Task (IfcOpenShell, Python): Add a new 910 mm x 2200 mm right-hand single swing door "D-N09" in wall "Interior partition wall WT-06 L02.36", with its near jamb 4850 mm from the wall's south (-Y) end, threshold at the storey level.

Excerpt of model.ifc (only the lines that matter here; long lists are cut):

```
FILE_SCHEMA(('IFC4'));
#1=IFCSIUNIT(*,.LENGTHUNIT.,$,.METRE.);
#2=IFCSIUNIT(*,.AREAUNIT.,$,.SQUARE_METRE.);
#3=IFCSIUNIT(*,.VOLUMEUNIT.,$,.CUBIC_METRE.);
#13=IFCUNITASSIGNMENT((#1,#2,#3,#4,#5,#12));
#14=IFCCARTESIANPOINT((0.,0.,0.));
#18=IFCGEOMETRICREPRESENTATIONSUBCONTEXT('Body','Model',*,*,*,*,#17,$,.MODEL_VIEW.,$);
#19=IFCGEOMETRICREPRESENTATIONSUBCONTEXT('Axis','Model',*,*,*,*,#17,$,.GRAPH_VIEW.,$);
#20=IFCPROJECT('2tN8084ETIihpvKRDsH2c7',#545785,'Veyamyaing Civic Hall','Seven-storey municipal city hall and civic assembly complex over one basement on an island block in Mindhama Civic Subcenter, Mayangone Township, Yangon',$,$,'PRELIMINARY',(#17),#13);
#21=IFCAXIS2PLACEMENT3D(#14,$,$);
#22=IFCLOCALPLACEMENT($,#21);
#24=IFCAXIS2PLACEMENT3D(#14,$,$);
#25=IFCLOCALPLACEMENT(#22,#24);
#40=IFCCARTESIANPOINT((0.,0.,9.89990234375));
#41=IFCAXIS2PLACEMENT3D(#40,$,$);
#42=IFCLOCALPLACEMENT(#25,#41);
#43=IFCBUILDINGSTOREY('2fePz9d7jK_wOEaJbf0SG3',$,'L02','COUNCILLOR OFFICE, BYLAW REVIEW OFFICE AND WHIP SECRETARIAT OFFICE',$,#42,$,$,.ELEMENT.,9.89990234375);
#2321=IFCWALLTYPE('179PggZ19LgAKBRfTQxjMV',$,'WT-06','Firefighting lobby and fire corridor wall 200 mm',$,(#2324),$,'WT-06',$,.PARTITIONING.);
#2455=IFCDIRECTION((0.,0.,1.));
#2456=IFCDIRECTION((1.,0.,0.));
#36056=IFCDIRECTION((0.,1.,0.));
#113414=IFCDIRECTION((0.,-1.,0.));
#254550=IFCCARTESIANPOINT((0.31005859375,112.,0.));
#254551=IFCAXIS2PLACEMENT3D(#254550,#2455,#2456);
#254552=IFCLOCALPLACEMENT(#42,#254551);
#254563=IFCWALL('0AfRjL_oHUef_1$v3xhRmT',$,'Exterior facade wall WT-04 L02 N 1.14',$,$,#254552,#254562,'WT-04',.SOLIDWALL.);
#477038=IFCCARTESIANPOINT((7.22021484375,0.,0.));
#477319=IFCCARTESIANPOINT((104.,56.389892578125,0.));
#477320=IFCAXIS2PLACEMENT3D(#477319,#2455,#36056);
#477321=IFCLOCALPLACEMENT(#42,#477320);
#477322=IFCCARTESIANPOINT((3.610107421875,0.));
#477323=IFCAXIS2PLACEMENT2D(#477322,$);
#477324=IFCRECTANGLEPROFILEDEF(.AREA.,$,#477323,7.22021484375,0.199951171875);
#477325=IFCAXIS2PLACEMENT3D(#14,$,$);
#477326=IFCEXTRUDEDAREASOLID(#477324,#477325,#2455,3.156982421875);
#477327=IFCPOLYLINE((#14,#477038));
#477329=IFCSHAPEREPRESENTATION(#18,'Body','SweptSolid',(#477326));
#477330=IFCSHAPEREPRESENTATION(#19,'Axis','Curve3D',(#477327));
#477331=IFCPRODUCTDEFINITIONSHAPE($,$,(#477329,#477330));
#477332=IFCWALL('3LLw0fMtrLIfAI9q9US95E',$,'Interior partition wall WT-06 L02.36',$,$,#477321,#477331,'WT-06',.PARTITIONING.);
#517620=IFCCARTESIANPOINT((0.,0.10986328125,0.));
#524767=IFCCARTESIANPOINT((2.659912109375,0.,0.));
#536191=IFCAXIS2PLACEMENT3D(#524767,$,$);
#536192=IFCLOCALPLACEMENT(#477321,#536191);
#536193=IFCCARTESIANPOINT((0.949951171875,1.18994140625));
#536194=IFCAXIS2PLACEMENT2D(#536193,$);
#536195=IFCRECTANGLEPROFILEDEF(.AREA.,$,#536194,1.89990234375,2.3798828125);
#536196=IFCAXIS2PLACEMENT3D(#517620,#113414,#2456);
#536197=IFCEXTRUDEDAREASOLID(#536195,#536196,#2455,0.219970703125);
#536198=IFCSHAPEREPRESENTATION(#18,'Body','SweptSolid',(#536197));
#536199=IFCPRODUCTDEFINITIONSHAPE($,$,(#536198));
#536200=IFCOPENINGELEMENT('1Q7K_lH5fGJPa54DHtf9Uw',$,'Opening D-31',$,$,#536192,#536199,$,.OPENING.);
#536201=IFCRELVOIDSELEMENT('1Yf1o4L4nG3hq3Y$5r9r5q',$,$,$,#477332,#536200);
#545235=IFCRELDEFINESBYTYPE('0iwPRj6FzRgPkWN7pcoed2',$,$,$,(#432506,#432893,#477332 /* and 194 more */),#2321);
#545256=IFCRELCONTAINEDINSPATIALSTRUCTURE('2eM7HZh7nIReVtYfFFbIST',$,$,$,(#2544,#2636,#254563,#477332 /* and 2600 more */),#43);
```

```python
import numpy as np
import ifcopenshell
import ifcopenshell.api.feature
import ifcopenshell.api.geometry
import ifcopenshell.api.root
import ifcopenshell.api.spatial
import ifcopenshell.geom
import ifcopenshell.util.element
import ifcopenshell.util.placement
import ifcopenshell.util.representation
import ifcopenshell.util.shape
import ifcopenshell.util.unit

model = ifcopenshell.open("model.ifc")
unit_scale = ifcopenshell.util.unit.calculate_unit_scale(model)
settings = ifcopenshell.geom.settings()


def volume(element):
    """Net volume in cubic metres, openings subtracted."""
    shape = ifcopenshell.geom.create_shape(settings, element)
    return ifcopenshell.util.shape.get_volume(shape.geometry)


wall = model.by_id(477332)
storey = ifcopenshell.util.element.get_container(wall, ifc_class="IfcBuildingStorey")
context = ifcopenshell.util.representation.get_context(model, "Model", "Body", "MODEL_VIEW")
before = volume(wall)

width, height, from_end, sill = 0.91, 2.2, 4.85, 0.0  # metres

# The wall runs along its own X axis, and the end named is its -X end.
wall_shape = ifcopenshell.geom.create_shape(settings, wall)
x, y, z = ifcopenshell.util.shape.get_vertices(wall_shape.geometry).T
start = x.min() + from_end
face, thickness = float(y.min()), float(y.max() - y.min())
wall_matrix = ifcopenshell.util.placement.get_local_placement(wall.ObjectPlacement)
level = ifcopenshell.util.placement.get_local_placement(storey.ObjectPlacement)[2, 3]


def in_wall(x, y):
    """Placement at x, y metres in the wall's axes, at sill height."""
    matrix = wall_matrix.copy()
    matrix[:, 3] = wall_matrix @ np.array([x / unit_scale, y / unit_scale, 0.0, 1.0])
    matrix[2, 3] = level + sill / unit_scale
    return matrix


# Opening: a box that overshoots both wall faces by 50 mm.
opening = ifcopenshell.api.root.create_entity(model, ifc_class="IfcOpeningElement", predefined_type="OPENING")
box = ifcopenshell.api.geometry.add_wall_representation(
    model, context=context, length=width, height=height, thickness=thickness + 0.1
)
ifcopenshell.api.geometry.assign_representation(model, product=opening, representation=box)
ifcopenshell.api.geometry.edit_object_placement(model, product=opening, matrix=in_wall(start, face - 0.05), is_si=False)
ifcopenshell.api.feature.add_feature(model, feature=opening, element=wall)

door = ifcopenshell.api.root.create_entity(model, ifc_class="IfcDoor", name="D-N09", predefined_type="DOOR")
door.OverallWidth, door.OverallHeight = width / unit_scale, height / unit_scale
door.OperationType = "SINGLE_SWING_RIGHT"
body = ifcopenshell.api.geometry.add_door_representation(
    model,
    context=context,
    overall_width=door.OverallWidth,
    overall_height=door.OverallHeight,
    operation_type="SINGLE_SWING_RIGHT",
    lining_properties={"LiningDepth": thickness / unit_scale, "ThresholdDepth": thickness / unit_scale},
)
ifcopenshell.api.geometry.assign_representation(model, product=door, representation=body)
ifcopenshell.api.spatial.assign_container(model, products=[door], relating_structure=storey)
ifcopenshell.api.feature.add_filling(model, opening=opening, element=door)

# The lining spans the wall, so the door starts at the wall face.
ifcopenshell.api.geometry.edit_object_placement(model, product=door, matrix=in_wall(start, face), is_si=False)

after = volume(wall)

print(f"wall volume {before:.3f} -> {after:.3f} m3")

model.write("model_updated.ifc")
```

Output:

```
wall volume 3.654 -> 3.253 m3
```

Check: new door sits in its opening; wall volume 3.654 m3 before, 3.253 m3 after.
